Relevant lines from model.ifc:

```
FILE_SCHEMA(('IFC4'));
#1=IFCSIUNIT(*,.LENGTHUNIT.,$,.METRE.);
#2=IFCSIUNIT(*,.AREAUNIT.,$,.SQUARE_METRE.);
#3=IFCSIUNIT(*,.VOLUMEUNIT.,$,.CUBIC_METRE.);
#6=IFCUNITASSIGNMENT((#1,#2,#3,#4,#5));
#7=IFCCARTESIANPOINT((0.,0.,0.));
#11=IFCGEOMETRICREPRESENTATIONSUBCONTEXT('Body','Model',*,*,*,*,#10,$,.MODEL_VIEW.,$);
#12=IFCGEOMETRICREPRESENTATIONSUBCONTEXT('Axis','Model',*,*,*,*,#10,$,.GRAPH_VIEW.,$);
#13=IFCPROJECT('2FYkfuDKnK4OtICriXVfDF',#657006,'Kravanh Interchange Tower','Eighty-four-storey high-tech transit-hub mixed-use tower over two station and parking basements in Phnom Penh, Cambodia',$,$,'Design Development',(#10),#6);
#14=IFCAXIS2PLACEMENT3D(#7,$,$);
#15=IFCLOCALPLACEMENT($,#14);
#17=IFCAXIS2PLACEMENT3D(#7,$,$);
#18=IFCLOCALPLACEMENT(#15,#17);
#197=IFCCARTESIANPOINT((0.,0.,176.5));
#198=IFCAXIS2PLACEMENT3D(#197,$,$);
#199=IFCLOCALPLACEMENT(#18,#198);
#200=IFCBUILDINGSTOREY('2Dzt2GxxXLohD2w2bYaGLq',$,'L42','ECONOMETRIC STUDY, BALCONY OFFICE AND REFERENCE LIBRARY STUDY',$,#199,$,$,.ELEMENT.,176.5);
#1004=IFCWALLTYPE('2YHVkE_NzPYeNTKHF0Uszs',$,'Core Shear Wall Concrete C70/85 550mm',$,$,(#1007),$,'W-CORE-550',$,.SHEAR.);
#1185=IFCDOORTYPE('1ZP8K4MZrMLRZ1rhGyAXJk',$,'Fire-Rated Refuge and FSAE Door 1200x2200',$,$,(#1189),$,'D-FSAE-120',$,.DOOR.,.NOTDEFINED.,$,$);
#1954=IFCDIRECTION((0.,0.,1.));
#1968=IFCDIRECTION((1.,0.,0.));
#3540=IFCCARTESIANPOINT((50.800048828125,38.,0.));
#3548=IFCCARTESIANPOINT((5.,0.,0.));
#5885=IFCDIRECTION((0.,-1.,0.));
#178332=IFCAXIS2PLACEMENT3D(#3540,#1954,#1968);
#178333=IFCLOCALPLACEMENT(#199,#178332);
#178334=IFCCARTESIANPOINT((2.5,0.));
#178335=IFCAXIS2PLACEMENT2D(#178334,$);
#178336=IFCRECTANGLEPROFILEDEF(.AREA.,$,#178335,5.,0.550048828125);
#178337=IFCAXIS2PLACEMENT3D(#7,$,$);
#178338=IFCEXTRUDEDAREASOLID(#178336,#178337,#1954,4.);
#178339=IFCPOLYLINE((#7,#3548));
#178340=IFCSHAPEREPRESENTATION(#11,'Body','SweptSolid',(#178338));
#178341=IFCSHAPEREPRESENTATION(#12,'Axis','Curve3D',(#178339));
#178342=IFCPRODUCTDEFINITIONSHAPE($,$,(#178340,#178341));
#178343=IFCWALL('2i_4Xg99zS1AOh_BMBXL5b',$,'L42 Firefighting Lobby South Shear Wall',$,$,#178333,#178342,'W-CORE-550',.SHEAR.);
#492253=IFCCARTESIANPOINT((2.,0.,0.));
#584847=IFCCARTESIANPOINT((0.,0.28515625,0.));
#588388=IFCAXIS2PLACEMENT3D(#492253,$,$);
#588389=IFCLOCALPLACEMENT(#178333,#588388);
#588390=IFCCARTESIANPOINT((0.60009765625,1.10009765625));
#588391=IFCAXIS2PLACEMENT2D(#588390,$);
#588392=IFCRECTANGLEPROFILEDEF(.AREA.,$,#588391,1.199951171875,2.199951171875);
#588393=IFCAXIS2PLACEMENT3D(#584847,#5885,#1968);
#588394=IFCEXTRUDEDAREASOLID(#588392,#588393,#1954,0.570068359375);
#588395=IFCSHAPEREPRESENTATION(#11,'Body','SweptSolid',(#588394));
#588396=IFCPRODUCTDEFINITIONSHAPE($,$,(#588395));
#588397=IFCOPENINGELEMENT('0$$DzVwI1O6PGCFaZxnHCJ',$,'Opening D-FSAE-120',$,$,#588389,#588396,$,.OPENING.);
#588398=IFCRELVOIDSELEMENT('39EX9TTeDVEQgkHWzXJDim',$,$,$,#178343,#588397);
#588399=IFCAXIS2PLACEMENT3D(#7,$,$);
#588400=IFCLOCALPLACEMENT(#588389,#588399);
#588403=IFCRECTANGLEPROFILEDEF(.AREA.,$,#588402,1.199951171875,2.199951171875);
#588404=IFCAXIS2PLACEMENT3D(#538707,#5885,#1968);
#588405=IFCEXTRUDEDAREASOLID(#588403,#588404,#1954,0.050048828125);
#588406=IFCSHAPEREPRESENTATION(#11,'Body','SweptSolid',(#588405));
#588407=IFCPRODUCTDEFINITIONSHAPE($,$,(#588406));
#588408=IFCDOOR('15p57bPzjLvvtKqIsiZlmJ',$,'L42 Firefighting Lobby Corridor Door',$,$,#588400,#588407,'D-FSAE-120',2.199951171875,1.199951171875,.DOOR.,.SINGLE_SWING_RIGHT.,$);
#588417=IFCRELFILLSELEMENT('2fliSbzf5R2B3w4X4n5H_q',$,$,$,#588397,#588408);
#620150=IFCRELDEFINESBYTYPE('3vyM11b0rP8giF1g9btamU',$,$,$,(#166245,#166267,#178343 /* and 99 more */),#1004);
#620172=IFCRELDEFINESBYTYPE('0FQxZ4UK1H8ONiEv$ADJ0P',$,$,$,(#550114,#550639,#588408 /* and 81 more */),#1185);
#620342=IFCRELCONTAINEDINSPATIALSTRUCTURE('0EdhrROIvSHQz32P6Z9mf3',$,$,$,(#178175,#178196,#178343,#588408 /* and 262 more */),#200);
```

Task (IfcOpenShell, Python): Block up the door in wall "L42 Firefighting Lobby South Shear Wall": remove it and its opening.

```python
import ifcopenshell
import ifcopenshell.api.feature
import ifcopenshell.api.root
import ifcopenshell.geom
import ifcopenshell.util.shape

model = ifcopenshell.open("model.ifc")
settings = ifcopenshell.geom.settings()


def volume(element):
    """Net volume in cubic metres, openings subtracted."""
    shape = ifcopenshell.geom.create_shape(settings, element)
    return ifcopenshell.util.shape.get_volume(shape.geometry)


door = model.by_guid("15p57bPzjLvvtKqIsiZlmJ")
opening = door.FillsVoids[0].RelatingOpeningElement
wall = opening.VoidsElements[0].RelatingBuildingElement
before = volume(wall)

ifcopenshell.api.root.remove_product(model, product=door)
ifcopenshell.api.feature.remove_feature(model, feature=opening)

after = volume(wall)

print(f"wall volume {before:.3f} -> {after:.3f} m3")

model.write("model_v2.ifc")
```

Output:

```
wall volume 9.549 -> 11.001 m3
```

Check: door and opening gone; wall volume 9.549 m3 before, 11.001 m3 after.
